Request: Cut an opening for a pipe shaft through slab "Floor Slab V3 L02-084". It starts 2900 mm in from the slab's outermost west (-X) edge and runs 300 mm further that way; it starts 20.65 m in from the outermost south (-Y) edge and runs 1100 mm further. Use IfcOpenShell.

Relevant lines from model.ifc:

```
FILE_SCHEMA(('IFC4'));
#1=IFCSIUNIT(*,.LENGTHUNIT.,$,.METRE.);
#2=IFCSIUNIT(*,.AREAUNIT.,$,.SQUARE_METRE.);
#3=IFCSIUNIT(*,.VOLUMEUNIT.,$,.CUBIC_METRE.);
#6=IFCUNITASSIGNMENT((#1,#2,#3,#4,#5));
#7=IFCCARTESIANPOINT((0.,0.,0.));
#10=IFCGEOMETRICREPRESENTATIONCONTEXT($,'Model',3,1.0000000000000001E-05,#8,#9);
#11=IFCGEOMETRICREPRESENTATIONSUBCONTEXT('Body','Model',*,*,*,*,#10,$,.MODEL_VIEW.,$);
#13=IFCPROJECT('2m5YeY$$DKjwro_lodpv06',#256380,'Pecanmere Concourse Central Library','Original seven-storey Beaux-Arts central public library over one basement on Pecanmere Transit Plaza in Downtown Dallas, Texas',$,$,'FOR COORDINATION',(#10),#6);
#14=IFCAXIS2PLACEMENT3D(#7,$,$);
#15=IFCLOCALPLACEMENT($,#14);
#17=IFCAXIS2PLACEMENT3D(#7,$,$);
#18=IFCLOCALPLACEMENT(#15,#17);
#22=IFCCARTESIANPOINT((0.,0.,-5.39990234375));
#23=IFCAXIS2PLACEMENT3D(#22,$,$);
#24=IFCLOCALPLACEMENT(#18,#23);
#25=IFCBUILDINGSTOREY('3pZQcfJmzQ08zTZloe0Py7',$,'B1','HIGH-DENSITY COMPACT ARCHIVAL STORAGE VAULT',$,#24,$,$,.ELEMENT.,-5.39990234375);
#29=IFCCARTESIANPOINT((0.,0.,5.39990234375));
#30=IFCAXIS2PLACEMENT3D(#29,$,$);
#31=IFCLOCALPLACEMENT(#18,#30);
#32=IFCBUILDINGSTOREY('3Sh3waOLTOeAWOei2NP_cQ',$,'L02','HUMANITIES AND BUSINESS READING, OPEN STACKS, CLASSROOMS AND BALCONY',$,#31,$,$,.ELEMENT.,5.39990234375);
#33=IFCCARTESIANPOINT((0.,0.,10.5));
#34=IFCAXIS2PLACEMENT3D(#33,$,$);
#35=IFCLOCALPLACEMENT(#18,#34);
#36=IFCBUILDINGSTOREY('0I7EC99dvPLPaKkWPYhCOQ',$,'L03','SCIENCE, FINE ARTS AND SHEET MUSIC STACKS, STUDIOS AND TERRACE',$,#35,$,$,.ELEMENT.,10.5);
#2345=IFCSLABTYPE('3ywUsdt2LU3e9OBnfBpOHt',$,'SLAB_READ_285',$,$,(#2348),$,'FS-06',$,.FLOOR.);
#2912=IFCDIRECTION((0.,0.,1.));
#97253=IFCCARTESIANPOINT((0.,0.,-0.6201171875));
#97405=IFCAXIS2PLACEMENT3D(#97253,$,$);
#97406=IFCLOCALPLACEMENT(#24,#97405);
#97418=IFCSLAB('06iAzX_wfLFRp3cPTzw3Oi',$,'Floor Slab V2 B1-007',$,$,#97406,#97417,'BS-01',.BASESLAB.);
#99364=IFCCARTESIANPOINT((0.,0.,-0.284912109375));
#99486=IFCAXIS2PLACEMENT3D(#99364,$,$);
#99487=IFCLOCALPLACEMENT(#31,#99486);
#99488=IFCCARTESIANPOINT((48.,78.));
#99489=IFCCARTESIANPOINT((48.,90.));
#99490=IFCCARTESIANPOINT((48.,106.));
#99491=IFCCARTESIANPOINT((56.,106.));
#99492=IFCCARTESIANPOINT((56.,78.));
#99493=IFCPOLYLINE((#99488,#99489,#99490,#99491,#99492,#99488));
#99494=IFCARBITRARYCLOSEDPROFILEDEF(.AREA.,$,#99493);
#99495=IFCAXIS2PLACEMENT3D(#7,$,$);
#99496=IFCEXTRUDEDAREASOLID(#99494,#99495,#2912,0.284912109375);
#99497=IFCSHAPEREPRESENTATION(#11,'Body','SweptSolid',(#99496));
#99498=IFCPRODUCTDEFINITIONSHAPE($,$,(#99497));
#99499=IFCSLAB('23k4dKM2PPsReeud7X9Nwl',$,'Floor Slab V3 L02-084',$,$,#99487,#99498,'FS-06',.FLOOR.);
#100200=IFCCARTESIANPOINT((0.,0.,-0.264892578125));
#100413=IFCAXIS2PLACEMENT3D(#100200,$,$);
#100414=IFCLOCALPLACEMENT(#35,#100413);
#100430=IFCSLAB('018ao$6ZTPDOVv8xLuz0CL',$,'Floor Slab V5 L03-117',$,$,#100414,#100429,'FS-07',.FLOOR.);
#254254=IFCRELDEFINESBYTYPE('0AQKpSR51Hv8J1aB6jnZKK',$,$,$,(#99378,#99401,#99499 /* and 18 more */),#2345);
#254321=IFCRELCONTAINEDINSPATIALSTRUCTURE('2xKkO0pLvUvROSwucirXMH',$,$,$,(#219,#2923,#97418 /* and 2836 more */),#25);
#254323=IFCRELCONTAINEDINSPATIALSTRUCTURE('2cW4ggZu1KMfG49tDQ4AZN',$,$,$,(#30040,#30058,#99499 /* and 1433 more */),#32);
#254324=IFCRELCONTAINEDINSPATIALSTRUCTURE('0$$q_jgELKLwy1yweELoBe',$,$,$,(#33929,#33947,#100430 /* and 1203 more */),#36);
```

```python
import numpy as np
import ifcopenshell
import ifcopenshell.api.feature
import ifcopenshell.api.geometry
import ifcopenshell.api.root
import ifcopenshell.geom
import ifcopenshell.util.placement
import ifcopenshell.util.representation
import ifcopenshell.util.shape
import ifcopenshell.util.unit

model = ifcopenshell.open("model.ifc")
unit_scale = ifcopenshell.util.unit.calculate_unit_scale(model)
settings = ifcopenshell.geom.settings()


def volume(element):
    """Net volume in cubic metres, openings subtracted."""
    shape = ifcopenshell.geom.create_shape(settings, element)
    return ifcopenshell.util.shape.get_volume(shape.geometry)


slab = model.by_id(99499)
before = volume(slab)

# Extent in the slab's own axes, in metres. The edges named are its -X and -Y sides.
slab_shape = ifcopenshell.geom.create_shape(settings, slab)
vertices = ifcopenshell.util.shape.get_vertices(slab_shape.geometry)
x_min, y_min, bottom = vertices.min(axis=0)
top = vertices[:, 2].max()

opening = ifcopenshell.api.root.create_entity(model, ifc_class="IfcOpeningElement", name="Pipe shaft opening", predefined_type="OPENING")
context = ifcopenshell.util.representation.get_context(model, "Model", "Body", "MODEL_VIEW")
width, depth = 0.3, 1.1
outline = [(0.0, 0.0), (width, 0.0), (width, depth), (0.0, depth), (0.0, 0.0)]
# Overshoot both faces by 50 mm so the cut is clean.
shape = ifcopenshell.api.geometry.add_slab_representation(
    model, context=context, depth=top - bottom + 0.1, polyline=outline
)
ifcopenshell.api.geometry.assign_representation(model, product=opening, representation=shape)

matrix = ifcopenshell.util.placement.get_local_placement(slab.ObjectPlacement)
matrix[:, 3] = matrix @ np.append(np.array([x_min + 2.9, y_min + 20.65, bottom - 0.05]) / unit_scale, 1.0)
ifcopenshell.api.geometry.edit_object_placement(model, product=opening, matrix=matrix, is_si=False)
ifcopenshell.api.feature.add_feature(model, feature=opening, element=slab)

after = volume(slab)

print(f"slab volume {before:.3f} -> {after:.3f} m3")

model.write("model_rev.ifc")
```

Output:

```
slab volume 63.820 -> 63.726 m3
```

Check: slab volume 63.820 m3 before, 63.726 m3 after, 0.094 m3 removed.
